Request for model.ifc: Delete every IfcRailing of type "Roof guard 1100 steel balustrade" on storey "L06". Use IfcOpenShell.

First a look at what the model holds.

```python
import ifcopenshell
import ifcopenshell.util.element

model = ifcopenshell.open("model.ifc")
print(model.schema)
storey = next(s for s in model.by_type("IfcBuildingStorey") if s.Name == "L06")
railings = [e for e in ifcopenshell.util.element.get_decomposition(storey) if e.is_a("IfcRailing")]
seen = {}
for e in railings:
    element_type = ifcopenshell.util.element.get_type(e)
    name = element_type.Name if element_type not in (None, e) else None
    seen[name] = seen.get(name, 0) + 1
for name, count in sorted(seen.items(), key=str):
    print(count, "x", name)
```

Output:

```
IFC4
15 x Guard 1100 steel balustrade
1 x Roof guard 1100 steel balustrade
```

```python
import ifcopenshell
import ifcopenshell.api.root
import ifcopenshell.util.element

model = ifcopenshell.open("model.ifc")

storey = next(s for s in model.by_type("IfcBuildingStorey") if s.Name == "L06")
railings = [e for e in ifcopenshell.util.element.get_decomposition(storey) if e.is_a("IfcRailing")]
targets = [e for e in railings if (t := ifcopenshell.util.element.get_type(e)) not in (None, e) and t.Name == "Roof guard 1100 steel balustrade"]

for e in targets:
    ifcopenshell.api.root.remove_product(model, product=e)
print(len(targets), "removed")

model.write("model-out.ifc")
```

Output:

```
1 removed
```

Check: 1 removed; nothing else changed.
